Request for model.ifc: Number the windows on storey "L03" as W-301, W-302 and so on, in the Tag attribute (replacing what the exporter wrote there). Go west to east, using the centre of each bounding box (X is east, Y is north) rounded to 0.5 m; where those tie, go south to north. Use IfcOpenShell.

First a look at what the model holds.

```python
import ifcopenshell
import ifcopenshell.util.element
import ifcopenshell.util.placement

model = ifcopenshell.open("model.ifc")
print(model.schema)
storey = next(s for s in model.by_type("IfcBuildingStorey") if s.Name == "L03")
windows = [e for e in ifcopenshell.util.element.get_decomposition(storey) if e.is_a("IfcWindow")]
for e in sorted(windows, key=lambda e: e.id()):
    origin = ifcopenshell.util.placement.get_local_placement(e.ObjectPlacement)[:3, 3]
    print(e.id(), e.Tag, e.Name, origin.round(2) + 0.0, sep=" | ")
```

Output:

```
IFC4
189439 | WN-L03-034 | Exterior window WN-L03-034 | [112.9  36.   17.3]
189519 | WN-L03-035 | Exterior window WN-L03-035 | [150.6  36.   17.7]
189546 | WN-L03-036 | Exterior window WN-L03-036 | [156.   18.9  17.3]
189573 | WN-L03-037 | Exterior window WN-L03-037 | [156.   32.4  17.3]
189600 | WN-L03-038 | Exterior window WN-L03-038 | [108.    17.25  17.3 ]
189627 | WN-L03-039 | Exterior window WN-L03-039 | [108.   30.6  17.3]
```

```python
import ifcopenshell
import ifcopenshell.geom
import ifcopenshell.util.element
import ifcopenshell.util.shape

model = ifcopenshell.open("model.ifc")
settings = ifcopenshell.geom.settings()
settings.set("use-world-coords", True)


def centre(element):
    shape = ifcopenshell.geom.create_shape(settings, element)
    return ifcopenshell.util.shape.get_bbox_centroid(shape.geometry)


storey = next(s for s in model.by_type("IfcBuildingStorey") if s.Name == "L03")
windows = [e for e in ifcopenshell.util.element.get_decomposition(storey) if e.is_a("IfcWindow")]

# Insertion points can sit at a corner or the storey origin, so sort by the geometry (in metres).
centres = {e: centre(e) for e in windows}
windows.sort(key=lambda e: (round(centres[e][0] / 0.5), centres[e][1]))

for i, e in enumerate(windows, start=1):
    number = f"W-3{i:02d}"
    e.Tag = number
    print(e.id(), number)

model.write("model_edited.ifc")
```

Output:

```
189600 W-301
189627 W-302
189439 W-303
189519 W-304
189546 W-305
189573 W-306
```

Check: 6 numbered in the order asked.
